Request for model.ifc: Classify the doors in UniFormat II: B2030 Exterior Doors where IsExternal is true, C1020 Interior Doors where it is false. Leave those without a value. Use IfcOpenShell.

First a look at what the model holds.

```python
import ifcopenshell
import ifcopenshell.util.element

model = ifcopenshell.open("model.ifc")
print(model.schema)
print("classifications:", [c.Name for c in model.by_type("IfcClassification")])
values = [ifcopenshell.util.element.get_pset(e, "Pset_DoorCommon", "IsExternal") for e in model.by_type("IfcDoor")]
for value in (True, False, None):
    print("IsExternal", value, values.count(value))
```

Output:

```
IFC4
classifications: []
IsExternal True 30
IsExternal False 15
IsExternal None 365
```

```python
import ifcopenshell
import ifcopenshell.api.classification
import ifcopenshell.util.element

model = ifcopenshell.open("model.ifc")

system = ifcopenshell.api.classification.add_classification(model, classification="UniFormat II")

doors = model.by_type("IfcDoor")
external = {e: ifcopenshell.util.element.get_pset(e, "Pset_DoorCommon", "IsExternal") for e in doors}
for flag, code, name in ((True, "B2030", "Exterior Doors"), (False, "C1020", "Interior Doors")):
    products = [e for e in doors if external[e] is flag]
    ifcopenshell.api.classification.add_reference(
        model, products=products, classification=system, identification=code, name=name
    )
    print(code, len(products))

model.write("model_updated.ifc")
```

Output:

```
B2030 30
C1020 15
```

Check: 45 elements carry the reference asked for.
